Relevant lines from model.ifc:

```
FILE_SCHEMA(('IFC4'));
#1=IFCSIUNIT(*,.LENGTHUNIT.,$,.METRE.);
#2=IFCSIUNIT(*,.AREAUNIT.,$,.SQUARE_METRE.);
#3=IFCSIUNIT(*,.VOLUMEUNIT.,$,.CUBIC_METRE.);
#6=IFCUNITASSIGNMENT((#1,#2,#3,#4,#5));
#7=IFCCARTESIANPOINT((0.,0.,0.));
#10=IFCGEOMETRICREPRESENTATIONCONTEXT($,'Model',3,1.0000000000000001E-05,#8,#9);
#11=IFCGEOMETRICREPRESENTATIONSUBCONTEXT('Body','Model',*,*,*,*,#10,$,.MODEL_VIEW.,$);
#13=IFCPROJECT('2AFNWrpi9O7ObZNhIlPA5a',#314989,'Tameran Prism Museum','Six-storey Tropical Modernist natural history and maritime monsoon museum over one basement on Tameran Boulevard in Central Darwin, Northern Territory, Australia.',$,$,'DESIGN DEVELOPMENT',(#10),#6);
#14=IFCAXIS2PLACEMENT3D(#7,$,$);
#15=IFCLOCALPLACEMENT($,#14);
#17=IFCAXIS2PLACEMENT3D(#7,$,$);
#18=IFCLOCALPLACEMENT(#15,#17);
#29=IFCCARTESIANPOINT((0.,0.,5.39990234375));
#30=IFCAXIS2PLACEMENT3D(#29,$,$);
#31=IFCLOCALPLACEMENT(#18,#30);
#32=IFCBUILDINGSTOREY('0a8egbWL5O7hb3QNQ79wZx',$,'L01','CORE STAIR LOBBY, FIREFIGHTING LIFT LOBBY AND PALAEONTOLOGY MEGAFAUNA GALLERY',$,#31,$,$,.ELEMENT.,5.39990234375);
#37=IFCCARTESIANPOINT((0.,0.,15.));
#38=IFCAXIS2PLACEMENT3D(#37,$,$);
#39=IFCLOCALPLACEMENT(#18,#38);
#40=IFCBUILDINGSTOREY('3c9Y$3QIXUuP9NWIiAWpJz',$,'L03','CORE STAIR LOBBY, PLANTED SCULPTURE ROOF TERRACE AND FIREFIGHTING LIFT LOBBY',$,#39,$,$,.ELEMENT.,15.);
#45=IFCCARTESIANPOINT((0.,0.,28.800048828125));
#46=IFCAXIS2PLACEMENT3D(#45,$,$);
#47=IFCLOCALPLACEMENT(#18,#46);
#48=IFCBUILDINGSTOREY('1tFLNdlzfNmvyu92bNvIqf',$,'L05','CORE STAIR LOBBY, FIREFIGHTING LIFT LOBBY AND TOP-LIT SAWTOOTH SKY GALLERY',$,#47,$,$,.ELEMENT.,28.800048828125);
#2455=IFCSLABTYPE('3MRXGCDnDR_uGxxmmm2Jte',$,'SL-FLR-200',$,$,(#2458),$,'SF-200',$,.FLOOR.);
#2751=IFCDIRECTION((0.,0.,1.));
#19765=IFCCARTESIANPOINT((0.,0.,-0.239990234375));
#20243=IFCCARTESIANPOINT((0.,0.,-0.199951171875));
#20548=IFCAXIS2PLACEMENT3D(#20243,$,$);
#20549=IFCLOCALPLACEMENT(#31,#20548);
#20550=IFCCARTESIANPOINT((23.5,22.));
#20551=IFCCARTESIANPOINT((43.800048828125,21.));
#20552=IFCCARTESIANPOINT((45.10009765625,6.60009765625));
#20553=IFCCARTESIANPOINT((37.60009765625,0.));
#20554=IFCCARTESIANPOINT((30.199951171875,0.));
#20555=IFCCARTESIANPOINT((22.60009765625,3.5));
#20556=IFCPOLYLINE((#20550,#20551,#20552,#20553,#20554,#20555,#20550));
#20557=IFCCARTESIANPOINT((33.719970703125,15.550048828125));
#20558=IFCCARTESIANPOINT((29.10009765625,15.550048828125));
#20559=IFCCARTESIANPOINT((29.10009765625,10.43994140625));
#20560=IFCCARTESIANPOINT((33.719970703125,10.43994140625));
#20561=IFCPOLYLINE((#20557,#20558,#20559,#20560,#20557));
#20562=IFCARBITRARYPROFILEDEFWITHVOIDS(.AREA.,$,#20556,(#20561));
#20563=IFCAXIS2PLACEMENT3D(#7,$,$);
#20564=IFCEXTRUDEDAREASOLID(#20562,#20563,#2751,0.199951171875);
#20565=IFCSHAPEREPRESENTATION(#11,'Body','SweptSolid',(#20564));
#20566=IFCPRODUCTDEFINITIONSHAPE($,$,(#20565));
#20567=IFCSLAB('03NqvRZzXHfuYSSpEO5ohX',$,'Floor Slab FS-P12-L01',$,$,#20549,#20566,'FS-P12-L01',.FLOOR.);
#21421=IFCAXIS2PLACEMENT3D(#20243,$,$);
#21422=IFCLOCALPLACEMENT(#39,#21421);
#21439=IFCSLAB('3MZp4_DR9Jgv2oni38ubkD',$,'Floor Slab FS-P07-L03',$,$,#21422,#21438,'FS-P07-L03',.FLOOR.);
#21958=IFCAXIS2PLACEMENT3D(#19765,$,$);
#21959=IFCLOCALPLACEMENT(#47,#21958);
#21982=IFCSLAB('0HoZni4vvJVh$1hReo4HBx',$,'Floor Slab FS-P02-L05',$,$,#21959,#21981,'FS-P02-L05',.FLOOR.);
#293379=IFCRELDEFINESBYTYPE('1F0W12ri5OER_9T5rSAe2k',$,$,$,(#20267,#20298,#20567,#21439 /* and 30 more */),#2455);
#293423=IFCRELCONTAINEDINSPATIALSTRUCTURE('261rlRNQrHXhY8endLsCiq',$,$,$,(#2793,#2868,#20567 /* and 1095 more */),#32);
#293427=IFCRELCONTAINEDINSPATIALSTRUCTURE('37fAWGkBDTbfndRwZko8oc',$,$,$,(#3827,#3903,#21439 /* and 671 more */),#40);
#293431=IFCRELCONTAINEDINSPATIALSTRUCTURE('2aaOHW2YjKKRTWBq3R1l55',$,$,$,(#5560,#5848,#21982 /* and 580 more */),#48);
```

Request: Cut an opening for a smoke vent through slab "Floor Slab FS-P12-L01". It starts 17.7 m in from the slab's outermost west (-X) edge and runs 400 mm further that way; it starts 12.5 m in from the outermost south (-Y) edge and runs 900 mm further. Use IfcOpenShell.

```python
import numpy as np
import ifcopenshell
import ifcopenshell.api.feature
import ifcopenshell.api.geometry
import ifcopenshell.api.root
import ifcopenshell.geom
import ifcopenshell.util.placement
import ifcopenshell.util.representation
import ifcopenshell.util.shape
import ifcopenshell.util.unit

model = ifcopenshell.open("model.ifc")
unit_scale = ifcopenshell.util.unit.calculate_unit_scale(model)
settings = ifcopenshell.geom.settings()


def volume(element):
    """Net volume in cubic metres, openings subtracted."""
    shape = ifcopenshell.geom.create_shape(settings, element)
    return ifcopenshell.util.shape.get_volume(shape.geometry)


slab = model.by_guid("03NqvRZzXHfuYSSpEO5ohX")
before = volume(slab)

# Extent in the slab's own axes, in metres. The edges named are its -X and -Y sides.
slab_shape = ifcopenshell.geom.create_shape(settings, slab)
vertices = ifcopenshell.util.shape.get_vertices(slab_shape.geometry)
x_min, y_min, bottom = vertices.min(axis=0)
top = vertices[:, 2].max()

opening = ifcopenshell.api.root.create_entity(model, ifc_class="IfcOpeningElement", name="Smoke vent opening", predefined_type="OPENING")
context = ifcopenshell.util.representation.get_context(model, "Model", "Body", "MODEL_VIEW")
width, depth = 0.4, 0.9
outline = [(0.0, 0.0), (width, 0.0), (width, depth), (0.0, depth), (0.0, 0.0)]
# Overshoot both faces by 50 mm so the cut is clean.
shape = ifcopenshell.api.geometry.add_slab_representation(
    model, context=context, depth=top - bottom + 0.1, polyline=outline
)
ifcopenshell.api.geometry.assign_representation(model, product=opening, representation=shape)

matrix = ifcopenshell.util.placement.get_local_placement(slab.ObjectPlacement)
matrix[:, 3] = matrix @ np.append(np.array([x_min + 17.7, y_min + 12.5, bottom - 0.05]) / unit_scale, 1.0)
ifcopenshell.api.geometry.edit_object_placement(model, product=opening, matrix=matrix, is_si=False)
ifcopenshell.api.feature.add_feature(model, feature=opening, element=slab)

after = volume(slab)

print(f"slab volume {before:.3f} -> {after:.3f} m3")

model.write("model_rev.ifc")
```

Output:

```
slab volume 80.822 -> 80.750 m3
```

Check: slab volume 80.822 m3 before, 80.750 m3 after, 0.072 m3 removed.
